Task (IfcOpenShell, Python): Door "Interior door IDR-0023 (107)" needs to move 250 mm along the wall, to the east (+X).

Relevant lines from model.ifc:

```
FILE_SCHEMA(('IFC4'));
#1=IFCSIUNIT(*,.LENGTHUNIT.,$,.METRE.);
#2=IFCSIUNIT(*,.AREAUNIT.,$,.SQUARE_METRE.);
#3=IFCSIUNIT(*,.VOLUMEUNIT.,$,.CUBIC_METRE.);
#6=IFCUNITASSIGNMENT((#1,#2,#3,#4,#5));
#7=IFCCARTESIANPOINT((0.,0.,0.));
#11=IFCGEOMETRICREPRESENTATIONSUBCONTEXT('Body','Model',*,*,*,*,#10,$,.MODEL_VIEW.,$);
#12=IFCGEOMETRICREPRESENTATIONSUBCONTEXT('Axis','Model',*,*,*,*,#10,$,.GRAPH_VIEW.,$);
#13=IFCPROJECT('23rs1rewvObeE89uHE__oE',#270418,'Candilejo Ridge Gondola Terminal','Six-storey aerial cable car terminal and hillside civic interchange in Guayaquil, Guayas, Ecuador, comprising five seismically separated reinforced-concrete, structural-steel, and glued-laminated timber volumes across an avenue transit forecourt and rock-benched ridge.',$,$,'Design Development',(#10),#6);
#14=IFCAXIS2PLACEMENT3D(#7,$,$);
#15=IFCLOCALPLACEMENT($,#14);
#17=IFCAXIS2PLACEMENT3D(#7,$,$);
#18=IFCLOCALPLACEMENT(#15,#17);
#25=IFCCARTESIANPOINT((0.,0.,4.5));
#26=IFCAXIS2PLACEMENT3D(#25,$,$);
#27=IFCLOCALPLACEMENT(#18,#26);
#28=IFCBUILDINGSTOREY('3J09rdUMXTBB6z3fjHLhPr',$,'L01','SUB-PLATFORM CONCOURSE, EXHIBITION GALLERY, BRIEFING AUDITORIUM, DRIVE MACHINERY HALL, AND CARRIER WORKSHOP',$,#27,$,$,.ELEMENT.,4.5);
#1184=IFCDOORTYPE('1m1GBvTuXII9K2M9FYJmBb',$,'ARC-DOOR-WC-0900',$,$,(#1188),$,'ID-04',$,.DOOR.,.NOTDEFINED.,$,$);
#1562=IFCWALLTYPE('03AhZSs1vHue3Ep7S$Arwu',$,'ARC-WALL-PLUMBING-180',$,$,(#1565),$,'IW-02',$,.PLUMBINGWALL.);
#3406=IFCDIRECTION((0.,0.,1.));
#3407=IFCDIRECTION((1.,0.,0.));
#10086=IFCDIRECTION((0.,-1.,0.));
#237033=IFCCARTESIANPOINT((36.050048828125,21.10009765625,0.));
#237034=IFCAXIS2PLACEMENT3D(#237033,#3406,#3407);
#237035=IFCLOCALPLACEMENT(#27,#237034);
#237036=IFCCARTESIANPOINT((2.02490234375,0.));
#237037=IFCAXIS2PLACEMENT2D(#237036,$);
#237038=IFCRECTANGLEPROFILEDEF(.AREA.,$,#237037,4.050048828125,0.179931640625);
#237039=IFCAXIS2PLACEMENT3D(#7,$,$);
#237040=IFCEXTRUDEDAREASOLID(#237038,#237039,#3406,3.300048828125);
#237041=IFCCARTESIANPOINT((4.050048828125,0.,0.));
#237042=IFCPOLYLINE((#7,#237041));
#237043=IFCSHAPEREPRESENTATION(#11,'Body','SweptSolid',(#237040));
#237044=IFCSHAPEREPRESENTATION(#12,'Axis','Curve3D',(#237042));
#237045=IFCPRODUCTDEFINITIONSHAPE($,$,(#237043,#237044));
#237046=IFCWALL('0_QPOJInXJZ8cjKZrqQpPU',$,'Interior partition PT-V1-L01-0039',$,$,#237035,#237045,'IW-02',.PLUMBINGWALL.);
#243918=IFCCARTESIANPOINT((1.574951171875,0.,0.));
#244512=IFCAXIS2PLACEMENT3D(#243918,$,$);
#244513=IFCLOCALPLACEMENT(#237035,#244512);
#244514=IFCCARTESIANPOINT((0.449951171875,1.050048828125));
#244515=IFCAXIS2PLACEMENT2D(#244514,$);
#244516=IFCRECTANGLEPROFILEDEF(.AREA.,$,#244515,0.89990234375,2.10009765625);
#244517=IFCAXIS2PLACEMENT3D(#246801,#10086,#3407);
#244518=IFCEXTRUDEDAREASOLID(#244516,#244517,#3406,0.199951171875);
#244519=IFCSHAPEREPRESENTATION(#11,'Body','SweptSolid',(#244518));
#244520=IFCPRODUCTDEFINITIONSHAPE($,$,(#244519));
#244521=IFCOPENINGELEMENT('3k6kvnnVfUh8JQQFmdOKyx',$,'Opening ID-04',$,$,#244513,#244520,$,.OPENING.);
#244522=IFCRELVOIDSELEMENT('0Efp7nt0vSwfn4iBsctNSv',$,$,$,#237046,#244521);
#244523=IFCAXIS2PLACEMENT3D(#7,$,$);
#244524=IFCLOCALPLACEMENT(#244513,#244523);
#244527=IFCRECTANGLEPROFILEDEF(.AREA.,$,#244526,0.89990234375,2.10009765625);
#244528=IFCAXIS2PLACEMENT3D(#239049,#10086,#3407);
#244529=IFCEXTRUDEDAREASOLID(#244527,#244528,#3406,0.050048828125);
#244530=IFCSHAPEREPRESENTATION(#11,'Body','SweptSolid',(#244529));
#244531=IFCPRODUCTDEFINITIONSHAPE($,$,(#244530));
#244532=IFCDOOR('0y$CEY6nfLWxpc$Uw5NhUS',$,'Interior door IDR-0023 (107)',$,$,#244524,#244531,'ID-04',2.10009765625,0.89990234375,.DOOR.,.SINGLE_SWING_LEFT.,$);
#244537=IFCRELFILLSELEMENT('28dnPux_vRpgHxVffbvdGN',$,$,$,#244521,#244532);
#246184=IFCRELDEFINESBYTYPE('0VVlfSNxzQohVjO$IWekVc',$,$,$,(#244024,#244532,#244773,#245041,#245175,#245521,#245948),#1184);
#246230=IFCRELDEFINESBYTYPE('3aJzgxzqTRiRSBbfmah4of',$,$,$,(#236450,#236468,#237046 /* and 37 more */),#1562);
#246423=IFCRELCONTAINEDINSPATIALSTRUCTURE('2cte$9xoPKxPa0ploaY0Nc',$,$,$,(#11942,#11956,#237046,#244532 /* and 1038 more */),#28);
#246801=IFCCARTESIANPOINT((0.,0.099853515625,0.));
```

```python
import ifcopenshell
import ifcopenshell.api.geometry
import ifcopenshell.util.placement
import ifcopenshell.util.unit

model = ifcopenshell.open("model.ifc")
unit_scale = ifcopenshell.util.unit.calculate_unit_scale(model)

door = model.by_id(244532)
opening = door.FillsVoids[0].RelatingOpeningElement
wall = opening.VoidsElements[0].RelatingBuildingElement

wall_matrix = ifcopenshell.util.placement.get_local_placement(wall.ObjectPlacement)
shift = wall_matrix[:3, 0] * 0.25 / unit_scale
before = ifcopenshell.util.placement.get_local_placement(door.ObjectPlacement)[:3, 3].copy()

# The door is placed relative to its opening, so it follows when the opening moves.
matrix = ifcopenshell.util.placement.get_local_placement(opening.ObjectPlacement)
matrix[:3, 3] += shift
ifcopenshell.api.geometry.edit_object_placement(
    model, product=opening, matrix=matrix, is_si=False, should_transform_children=True
)

after = ifcopenshell.util.placement.get_local_placement(door.ObjectPlacement)[:3, 3]
print("door moved by", (after - before).round(3) + 0.0)

model.write("model-out.ifc")
```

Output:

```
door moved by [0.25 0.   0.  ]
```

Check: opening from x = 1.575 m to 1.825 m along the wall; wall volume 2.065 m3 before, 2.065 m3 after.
